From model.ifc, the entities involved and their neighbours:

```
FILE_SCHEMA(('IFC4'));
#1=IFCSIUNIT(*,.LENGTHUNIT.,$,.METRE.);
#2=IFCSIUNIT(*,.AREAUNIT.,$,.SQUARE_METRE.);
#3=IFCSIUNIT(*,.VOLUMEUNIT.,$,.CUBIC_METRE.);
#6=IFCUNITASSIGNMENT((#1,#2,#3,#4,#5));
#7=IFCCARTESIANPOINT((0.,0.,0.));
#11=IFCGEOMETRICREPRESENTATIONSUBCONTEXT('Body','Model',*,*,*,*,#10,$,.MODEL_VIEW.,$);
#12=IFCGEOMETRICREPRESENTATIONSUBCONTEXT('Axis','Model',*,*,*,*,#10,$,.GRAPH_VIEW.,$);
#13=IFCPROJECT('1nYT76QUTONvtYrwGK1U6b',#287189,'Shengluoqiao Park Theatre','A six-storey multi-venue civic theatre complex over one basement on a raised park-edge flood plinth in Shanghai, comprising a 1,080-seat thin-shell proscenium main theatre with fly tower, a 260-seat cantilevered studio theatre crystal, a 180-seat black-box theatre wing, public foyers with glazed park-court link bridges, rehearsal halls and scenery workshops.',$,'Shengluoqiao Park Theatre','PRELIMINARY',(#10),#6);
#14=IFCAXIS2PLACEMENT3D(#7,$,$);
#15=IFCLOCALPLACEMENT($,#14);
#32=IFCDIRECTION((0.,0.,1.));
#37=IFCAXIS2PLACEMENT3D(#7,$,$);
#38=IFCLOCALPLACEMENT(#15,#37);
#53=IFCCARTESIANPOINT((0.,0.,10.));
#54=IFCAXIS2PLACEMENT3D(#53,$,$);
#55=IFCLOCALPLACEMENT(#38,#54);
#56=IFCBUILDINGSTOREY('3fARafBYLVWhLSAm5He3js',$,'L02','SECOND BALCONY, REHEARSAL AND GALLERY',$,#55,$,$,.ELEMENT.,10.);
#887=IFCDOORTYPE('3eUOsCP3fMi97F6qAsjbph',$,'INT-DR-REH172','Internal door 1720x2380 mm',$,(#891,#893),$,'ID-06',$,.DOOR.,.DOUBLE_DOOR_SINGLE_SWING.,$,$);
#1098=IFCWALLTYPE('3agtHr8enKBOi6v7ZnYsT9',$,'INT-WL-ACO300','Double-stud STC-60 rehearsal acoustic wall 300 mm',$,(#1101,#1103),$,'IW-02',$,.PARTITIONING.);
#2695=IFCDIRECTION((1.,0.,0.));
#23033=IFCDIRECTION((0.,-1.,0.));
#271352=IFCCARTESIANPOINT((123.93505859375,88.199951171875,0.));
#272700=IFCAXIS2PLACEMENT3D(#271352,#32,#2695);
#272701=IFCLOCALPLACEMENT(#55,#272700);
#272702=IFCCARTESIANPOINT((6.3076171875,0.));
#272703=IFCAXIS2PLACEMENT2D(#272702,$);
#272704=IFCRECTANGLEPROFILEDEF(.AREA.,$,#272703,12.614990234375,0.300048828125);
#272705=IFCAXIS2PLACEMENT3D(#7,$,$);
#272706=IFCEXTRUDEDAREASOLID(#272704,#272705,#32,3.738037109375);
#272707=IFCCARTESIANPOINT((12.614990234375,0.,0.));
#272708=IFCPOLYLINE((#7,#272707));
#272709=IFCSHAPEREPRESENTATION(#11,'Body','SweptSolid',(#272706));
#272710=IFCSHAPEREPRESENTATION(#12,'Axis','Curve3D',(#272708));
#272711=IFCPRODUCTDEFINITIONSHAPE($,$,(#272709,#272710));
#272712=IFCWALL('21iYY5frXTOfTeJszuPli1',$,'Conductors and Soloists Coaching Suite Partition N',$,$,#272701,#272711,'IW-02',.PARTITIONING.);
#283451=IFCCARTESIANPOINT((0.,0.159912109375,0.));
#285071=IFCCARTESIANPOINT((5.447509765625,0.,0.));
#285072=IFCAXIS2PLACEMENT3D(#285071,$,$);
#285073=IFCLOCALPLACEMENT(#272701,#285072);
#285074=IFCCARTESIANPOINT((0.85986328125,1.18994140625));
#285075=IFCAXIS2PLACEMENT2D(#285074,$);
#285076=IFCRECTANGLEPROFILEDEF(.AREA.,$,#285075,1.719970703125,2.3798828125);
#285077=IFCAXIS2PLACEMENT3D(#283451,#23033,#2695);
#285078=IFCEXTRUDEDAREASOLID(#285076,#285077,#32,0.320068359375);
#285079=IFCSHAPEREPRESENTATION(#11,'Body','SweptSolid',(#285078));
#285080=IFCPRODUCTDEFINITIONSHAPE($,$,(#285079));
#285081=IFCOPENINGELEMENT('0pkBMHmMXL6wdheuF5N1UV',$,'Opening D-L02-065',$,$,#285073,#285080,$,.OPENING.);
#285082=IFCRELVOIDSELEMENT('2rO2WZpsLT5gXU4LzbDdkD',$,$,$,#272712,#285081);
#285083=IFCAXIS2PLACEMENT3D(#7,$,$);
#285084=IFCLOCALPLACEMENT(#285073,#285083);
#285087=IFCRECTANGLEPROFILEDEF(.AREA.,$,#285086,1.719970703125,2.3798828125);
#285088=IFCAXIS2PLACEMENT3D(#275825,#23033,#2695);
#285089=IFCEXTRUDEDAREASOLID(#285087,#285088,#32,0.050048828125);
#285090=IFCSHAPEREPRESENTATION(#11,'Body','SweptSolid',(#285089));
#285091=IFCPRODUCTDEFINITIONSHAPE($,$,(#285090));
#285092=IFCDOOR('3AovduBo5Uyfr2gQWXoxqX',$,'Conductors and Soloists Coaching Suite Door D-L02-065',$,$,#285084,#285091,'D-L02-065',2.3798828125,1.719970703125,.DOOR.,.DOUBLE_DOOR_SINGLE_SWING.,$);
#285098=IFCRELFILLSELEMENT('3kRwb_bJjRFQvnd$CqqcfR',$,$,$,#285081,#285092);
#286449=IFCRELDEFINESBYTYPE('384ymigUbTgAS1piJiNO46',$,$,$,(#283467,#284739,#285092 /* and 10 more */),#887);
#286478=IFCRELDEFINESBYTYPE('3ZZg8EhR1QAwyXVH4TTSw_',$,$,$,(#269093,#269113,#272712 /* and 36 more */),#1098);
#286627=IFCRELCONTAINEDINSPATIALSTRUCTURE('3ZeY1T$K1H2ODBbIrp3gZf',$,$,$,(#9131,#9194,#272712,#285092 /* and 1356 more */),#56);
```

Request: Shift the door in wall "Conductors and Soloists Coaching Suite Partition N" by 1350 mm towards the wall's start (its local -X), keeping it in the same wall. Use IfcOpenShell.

```python
import ifcopenshell
import ifcopenshell.api.geometry
import ifcopenshell.util.placement
import ifcopenshell.util.unit

model = ifcopenshell.open("model.ifc")
unit_scale = ifcopenshell.util.unit.calculate_unit_scale(model)

door = model.by_guid("3AovduBo5Uyfr2gQWXoxqX")
opening = door.FillsVoids[0].RelatingOpeningElement
wall = opening.VoidsElements[0].RelatingBuildingElement

wall_matrix = ifcopenshell.util.placement.get_local_placement(wall.ObjectPlacement)
shift = wall_matrix[:3, 0] * -1.35 / unit_scale
before = ifcopenshell.util.placement.get_local_placement(door.ObjectPlacement)[:3, 3].copy()

# The door is placed relative to its opening, so it follows when the opening moves.
matrix = ifcopenshell.util.placement.get_local_placement(opening.ObjectPlacement)
matrix[:3, 3] += shift
ifcopenshell.api.geometry.edit_object_placement(
    model, product=opening, matrix=matrix, is_si=False, should_transform_children=True
)

after = ifcopenshell.util.placement.get_local_placement(door.ObjectPlacement)[:3, 3]
print("door moved by", (after - before).round(3) + 0.0)

model.write("model_updated.ifc")
```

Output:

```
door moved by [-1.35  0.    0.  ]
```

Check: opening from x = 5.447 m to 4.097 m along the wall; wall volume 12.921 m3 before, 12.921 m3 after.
